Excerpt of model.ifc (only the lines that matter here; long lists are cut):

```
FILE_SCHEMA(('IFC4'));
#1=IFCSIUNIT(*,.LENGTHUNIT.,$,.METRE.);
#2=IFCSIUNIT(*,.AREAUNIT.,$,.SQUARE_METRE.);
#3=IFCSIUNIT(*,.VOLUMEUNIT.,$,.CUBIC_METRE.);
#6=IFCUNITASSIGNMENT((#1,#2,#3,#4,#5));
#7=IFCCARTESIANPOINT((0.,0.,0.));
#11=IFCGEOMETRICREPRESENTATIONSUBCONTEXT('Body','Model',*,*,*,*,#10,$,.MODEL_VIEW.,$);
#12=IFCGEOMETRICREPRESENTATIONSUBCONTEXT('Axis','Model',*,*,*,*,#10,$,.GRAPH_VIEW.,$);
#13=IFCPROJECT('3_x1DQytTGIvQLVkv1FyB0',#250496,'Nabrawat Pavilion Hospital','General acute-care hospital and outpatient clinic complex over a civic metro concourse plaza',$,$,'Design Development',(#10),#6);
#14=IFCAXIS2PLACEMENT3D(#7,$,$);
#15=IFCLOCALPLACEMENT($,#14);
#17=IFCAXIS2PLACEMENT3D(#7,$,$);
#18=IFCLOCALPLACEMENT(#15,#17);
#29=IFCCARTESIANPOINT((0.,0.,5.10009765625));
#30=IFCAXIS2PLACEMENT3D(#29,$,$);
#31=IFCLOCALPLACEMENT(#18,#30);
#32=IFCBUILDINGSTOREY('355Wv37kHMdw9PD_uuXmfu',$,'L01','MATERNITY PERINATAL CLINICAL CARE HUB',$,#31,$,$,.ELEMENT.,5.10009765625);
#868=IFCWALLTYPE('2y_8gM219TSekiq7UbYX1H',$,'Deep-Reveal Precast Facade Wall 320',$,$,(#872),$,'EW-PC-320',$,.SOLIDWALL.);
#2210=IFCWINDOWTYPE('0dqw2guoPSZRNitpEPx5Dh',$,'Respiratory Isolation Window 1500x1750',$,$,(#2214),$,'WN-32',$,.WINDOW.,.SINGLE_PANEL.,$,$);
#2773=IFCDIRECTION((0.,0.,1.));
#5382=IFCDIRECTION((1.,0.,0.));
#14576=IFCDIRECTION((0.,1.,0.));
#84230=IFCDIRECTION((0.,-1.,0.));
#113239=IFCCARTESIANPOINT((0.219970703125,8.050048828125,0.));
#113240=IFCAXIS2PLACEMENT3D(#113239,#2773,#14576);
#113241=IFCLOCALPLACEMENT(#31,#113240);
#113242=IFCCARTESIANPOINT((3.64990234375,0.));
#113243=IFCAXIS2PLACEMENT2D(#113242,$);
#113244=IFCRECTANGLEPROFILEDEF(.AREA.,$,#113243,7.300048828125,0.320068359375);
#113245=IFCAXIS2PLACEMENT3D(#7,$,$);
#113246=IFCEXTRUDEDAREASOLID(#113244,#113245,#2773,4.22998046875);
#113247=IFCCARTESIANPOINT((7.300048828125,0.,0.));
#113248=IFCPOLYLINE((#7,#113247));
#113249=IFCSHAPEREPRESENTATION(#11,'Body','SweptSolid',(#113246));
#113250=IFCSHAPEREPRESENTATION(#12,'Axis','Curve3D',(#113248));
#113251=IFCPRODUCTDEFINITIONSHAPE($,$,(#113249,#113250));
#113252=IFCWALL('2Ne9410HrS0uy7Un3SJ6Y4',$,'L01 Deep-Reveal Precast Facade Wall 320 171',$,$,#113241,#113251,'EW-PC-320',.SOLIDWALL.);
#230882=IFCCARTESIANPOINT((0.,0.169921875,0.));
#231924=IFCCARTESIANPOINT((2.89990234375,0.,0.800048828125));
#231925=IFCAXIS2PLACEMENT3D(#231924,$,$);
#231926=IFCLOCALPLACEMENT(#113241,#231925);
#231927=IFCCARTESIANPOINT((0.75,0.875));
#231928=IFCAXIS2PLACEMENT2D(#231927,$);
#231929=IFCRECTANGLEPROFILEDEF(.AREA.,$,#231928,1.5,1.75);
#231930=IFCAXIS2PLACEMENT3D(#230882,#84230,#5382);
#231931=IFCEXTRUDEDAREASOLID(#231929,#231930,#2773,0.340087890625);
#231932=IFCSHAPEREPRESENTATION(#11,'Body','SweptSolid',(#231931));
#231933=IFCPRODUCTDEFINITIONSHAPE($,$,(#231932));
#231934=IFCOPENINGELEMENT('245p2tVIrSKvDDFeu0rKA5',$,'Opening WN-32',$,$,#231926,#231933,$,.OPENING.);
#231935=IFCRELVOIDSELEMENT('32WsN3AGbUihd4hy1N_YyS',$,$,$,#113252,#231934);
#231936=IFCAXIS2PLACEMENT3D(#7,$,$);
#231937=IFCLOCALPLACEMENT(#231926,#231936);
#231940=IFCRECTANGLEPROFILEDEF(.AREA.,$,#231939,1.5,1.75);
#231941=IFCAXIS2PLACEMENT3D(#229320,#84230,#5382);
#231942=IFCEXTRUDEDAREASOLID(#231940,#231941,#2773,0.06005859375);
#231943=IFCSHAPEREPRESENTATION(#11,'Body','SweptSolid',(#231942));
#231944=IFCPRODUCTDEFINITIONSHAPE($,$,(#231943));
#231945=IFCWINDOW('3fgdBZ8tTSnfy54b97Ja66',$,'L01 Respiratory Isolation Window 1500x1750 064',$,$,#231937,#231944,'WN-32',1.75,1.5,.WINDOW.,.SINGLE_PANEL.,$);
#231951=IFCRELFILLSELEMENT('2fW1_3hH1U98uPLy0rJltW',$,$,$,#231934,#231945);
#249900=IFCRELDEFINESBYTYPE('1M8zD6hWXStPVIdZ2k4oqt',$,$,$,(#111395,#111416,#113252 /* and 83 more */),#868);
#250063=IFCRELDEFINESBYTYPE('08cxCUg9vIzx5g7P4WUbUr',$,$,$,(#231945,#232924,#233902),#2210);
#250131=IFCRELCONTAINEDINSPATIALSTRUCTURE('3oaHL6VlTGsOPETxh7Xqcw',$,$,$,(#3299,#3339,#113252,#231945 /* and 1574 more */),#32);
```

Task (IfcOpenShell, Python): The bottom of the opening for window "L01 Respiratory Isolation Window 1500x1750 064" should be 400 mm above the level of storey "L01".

```python
import numpy as np
import ifcopenshell
import ifcopenshell.api.geometry
import ifcopenshell.geom
import ifcopenshell.util.element
import ifcopenshell.util.placement
import ifcopenshell.util.shape
import ifcopenshell.util.unit

model = ifcopenshell.open("model.ifc")
unit_scale = ifcopenshell.util.unit.calculate_unit_scale(model)

window = model.by_id(231945)
opening = window.FillsVoids[0].RelatingOpeningElement
storey = ifcopenshell.util.element.get_container(window, ifc_class="IfcBuildingStorey")
level = ifcopenshell.util.placement.get_local_placement(storey.ObjectPlacement)[2, 3]

# The opening's origin need not be at the sill, so measure its lowest point.
shape = ifcopenshell.geom.create_shape(ifcopenshell.geom.settings(), opening)
bottom = ifcopenshell.util.shape.get_shape_bottom_elevation(shape, shape.geometry) / unit_scale
dz = level + 0.4 - bottom

shift = np.array([0.0, 0.0, dz])
# The window is placed relative to its opening, so it follows when the opening moves.
matrix = ifcopenshell.util.placement.get_local_placement(opening.ObjectPlacement)
matrix[:3, 3] += shift
ifcopenshell.api.geometry.edit_object_placement(
    model, product=opening, matrix=matrix, is_si=False, should_transform_children=True
)

print(f"moved by {dz * unit_scale:+.3f} m")

model.write("model_edited.ifc")
```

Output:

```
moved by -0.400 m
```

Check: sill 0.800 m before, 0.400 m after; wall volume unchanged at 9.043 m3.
